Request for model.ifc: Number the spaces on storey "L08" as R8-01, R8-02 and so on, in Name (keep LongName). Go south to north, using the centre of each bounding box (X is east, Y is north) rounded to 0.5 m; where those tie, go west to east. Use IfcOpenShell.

First a look at what the model holds.

```python
import ifcopenshell
import ifcopenshell.util.element
import ifcopenshell.util.placement

model = ifcopenshell.open("model.ifc")
print(model.schema)
storey = next(s for s in model.by_type("IfcBuildingStorey") if s.Name == "L08")
spaces = [e for e in ifcopenshell.util.element.get_decomposition(storey) if e.is_a("IfcSpace")]
for e in sorted(spaces, key=lambda e: e.id()):
    origin = ifcopenshell.util.placement.get_local_placement(e.ObjectPlacement)[:3, 3]
    print(e.id(), e.Name, e.LongName, origin.round(2) + 0.0, sep=" | ")
```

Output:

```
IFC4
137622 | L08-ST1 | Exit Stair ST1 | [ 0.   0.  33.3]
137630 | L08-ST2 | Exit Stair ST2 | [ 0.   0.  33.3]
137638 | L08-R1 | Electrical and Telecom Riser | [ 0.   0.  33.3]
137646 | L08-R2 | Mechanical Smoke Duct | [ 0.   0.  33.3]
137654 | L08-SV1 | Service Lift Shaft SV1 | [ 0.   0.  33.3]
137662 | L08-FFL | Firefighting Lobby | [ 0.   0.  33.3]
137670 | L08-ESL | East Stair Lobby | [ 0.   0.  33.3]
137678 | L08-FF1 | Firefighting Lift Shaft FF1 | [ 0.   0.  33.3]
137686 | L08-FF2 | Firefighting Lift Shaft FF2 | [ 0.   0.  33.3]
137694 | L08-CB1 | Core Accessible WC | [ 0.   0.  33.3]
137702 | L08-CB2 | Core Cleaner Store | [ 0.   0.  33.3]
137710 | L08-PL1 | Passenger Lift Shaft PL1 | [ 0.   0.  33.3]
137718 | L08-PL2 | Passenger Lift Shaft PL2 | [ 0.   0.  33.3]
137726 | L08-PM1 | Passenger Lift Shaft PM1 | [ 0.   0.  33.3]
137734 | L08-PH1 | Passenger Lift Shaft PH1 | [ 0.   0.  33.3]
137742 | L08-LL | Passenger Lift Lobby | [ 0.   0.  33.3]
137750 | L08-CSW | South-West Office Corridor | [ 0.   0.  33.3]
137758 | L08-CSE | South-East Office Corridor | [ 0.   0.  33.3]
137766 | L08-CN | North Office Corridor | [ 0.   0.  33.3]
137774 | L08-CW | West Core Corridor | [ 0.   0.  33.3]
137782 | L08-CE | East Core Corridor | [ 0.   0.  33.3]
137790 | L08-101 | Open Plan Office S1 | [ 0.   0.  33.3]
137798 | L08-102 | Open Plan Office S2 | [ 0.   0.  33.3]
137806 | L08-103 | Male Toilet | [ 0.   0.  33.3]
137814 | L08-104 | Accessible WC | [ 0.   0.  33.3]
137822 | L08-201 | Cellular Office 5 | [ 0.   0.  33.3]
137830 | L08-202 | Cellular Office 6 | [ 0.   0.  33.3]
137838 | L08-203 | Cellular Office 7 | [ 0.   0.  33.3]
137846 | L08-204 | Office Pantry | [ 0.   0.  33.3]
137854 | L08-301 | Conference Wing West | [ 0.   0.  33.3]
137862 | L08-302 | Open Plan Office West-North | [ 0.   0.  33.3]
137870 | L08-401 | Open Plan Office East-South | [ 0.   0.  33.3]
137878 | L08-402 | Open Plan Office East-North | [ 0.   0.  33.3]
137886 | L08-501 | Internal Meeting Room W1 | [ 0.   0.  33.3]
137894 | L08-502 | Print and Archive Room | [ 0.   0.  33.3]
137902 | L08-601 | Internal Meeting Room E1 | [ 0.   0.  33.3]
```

```python
import ifcopenshell
import ifcopenshell.geom
import ifcopenshell.util.element
import ifcopenshell.util.shape

model = ifcopenshell.open("model.ifc")
settings = ifcopenshell.geom.settings()
settings.set("use-world-coords", True)


def centre(element):
    shape = ifcopenshell.geom.create_shape(settings, element)
    return ifcopenshell.util.shape.get_bbox_centroid(shape.geometry)


storey = next(s for s in model.by_type("IfcBuildingStorey") if s.Name == "L08")
spaces = [e for e in ifcopenshell.util.element.get_decomposition(storey) if e.is_a("IfcSpace")]

# Insertion points can sit at a corner or the storey origin, so sort by the geometry (in metres).
centres = {e: centre(e) for e in spaces}
spaces.sort(key=lambda e: (round(centres[e][1] / 0.5), centres[e][0]))

for i, e in enumerate(spaces, start=1):
    number = f"R8-{i:02d}"
    e.Name = number
    print(e.id(), number)

model.write("model-out.ifc")
```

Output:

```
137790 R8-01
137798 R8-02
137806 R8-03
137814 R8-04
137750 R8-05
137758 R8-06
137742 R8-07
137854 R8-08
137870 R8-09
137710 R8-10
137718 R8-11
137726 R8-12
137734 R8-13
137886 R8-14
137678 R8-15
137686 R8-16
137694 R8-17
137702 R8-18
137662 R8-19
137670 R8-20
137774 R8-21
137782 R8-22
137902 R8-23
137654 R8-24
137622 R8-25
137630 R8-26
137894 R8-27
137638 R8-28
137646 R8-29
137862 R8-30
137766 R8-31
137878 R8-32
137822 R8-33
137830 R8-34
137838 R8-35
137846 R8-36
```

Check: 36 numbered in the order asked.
